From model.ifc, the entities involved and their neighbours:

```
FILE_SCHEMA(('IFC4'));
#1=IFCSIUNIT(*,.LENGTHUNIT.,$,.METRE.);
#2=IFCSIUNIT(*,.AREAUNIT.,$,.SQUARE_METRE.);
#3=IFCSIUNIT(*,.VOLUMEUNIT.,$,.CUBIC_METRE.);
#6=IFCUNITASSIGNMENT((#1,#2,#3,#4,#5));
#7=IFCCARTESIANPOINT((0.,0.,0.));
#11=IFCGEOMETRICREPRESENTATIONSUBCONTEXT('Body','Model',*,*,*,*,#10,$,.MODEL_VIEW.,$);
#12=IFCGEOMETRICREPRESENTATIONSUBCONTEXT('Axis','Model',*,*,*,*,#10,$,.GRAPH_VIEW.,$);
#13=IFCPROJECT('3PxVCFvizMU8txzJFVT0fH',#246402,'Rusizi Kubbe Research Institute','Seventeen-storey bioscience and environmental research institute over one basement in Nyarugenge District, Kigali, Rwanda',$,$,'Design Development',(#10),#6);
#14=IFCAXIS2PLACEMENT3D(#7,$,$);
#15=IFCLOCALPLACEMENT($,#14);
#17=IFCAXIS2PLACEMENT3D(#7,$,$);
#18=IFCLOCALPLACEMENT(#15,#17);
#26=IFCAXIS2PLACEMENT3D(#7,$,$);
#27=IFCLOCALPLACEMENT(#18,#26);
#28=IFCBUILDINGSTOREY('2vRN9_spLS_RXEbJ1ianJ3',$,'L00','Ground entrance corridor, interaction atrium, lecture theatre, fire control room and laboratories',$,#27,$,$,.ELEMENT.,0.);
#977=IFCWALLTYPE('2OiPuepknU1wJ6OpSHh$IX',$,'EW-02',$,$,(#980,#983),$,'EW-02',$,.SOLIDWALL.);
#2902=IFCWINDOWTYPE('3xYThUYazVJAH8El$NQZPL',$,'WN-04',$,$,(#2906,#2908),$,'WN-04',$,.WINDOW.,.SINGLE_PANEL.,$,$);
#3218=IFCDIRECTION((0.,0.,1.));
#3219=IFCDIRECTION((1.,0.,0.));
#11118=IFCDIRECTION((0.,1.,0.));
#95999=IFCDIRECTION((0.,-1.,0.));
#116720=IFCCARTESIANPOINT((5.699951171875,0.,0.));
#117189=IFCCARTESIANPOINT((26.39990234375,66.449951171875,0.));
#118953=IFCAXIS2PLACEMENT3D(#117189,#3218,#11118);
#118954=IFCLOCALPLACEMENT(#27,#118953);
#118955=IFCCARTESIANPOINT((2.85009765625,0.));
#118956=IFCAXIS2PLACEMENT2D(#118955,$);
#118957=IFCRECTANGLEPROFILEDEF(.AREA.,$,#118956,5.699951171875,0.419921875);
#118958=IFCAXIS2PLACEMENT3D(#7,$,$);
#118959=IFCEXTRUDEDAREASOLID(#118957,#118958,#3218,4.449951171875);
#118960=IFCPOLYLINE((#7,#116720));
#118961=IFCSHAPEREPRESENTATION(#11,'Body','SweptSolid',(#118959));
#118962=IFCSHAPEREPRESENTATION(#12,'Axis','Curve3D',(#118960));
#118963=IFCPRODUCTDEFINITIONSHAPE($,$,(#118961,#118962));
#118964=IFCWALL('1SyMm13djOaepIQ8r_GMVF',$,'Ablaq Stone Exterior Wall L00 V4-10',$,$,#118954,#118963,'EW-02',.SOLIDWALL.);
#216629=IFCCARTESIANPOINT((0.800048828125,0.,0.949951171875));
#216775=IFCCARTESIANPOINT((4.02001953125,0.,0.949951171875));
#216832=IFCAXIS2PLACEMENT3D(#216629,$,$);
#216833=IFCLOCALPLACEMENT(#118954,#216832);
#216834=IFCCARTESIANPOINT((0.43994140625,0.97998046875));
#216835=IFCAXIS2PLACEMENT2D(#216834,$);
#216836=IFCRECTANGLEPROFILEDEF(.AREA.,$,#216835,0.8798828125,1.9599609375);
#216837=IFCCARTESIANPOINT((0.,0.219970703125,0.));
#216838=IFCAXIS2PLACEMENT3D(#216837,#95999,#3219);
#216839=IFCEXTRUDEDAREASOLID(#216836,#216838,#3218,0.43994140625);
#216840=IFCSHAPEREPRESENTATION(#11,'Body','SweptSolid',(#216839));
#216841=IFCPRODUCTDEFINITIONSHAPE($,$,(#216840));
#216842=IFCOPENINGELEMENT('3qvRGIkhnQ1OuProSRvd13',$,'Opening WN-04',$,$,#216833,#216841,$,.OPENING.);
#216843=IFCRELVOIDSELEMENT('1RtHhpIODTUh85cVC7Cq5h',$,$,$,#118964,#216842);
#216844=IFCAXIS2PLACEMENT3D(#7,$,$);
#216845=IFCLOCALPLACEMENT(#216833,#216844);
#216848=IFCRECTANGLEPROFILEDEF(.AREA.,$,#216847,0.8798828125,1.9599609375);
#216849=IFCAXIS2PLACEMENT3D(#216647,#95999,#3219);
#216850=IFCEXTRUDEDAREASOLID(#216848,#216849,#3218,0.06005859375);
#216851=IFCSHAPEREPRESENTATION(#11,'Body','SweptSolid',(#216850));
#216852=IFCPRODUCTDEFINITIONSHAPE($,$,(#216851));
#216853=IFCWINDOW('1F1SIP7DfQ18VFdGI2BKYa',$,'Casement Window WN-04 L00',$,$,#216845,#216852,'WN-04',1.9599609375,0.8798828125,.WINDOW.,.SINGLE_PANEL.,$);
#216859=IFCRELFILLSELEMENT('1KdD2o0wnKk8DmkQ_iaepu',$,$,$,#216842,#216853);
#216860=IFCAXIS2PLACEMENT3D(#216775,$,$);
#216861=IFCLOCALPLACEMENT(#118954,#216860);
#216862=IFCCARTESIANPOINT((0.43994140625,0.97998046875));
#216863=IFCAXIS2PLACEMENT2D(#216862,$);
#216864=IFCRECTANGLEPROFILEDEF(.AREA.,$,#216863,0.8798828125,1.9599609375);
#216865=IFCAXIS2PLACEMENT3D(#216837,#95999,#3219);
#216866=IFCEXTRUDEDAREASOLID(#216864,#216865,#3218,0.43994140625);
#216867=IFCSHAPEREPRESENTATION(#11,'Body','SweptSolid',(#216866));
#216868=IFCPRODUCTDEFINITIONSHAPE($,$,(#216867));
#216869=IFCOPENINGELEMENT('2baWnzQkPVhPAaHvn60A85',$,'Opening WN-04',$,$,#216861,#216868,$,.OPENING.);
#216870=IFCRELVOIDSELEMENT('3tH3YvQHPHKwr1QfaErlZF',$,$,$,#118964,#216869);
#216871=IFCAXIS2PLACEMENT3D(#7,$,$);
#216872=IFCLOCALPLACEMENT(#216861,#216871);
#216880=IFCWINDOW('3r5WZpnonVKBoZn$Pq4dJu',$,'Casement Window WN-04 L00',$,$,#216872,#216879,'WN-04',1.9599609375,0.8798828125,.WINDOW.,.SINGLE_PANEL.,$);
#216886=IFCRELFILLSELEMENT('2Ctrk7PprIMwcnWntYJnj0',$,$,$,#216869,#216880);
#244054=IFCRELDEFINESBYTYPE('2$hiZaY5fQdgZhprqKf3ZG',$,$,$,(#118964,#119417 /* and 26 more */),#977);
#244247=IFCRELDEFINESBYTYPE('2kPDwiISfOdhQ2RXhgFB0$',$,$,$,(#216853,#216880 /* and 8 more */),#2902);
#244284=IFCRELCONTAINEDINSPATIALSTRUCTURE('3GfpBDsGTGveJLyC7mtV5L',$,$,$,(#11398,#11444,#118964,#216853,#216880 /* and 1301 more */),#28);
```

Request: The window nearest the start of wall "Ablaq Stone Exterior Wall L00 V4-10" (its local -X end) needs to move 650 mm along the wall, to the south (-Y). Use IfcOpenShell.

```python
import ifcopenshell
import ifcopenshell.api.geometry
import ifcopenshell.util.placement

model = ifcopenshell.open("model.ifc")

window = model.by_guid("1F1SIP7DfQ18VFdGI2BKYa")
opening = window.FillsVoids[0].RelatingOpeningElement
wall = opening.VoidsElements[0].RelatingBuildingElement

wall_matrix = ifcopenshell.util.placement.get_local_placement(wall.ObjectPlacement)
shift = wall_matrix[:3, 0] * -0.65
before = ifcopenshell.util.placement.get_local_placement(window.ObjectPlacement)[:3, 3].copy()

# The window is placed relative to its opening, so it follows when the opening moves.
matrix = ifcopenshell.util.placement.get_local_placement(opening.ObjectPlacement)
matrix[:3, 3] += shift
ifcopenshell.api.geometry.edit_object_placement(
    model, product=opening, matrix=matrix, is_si=False, should_transform_children=True
)

after = ifcopenshell.util.placement.get_local_placement(window.ObjectPlacement)[:3, 3]
print("window moved by", (after - before).round(3) + 0.0)

model.write("model-out.ifc")
```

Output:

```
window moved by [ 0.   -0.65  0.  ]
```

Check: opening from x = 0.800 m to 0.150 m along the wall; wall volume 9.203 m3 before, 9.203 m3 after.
